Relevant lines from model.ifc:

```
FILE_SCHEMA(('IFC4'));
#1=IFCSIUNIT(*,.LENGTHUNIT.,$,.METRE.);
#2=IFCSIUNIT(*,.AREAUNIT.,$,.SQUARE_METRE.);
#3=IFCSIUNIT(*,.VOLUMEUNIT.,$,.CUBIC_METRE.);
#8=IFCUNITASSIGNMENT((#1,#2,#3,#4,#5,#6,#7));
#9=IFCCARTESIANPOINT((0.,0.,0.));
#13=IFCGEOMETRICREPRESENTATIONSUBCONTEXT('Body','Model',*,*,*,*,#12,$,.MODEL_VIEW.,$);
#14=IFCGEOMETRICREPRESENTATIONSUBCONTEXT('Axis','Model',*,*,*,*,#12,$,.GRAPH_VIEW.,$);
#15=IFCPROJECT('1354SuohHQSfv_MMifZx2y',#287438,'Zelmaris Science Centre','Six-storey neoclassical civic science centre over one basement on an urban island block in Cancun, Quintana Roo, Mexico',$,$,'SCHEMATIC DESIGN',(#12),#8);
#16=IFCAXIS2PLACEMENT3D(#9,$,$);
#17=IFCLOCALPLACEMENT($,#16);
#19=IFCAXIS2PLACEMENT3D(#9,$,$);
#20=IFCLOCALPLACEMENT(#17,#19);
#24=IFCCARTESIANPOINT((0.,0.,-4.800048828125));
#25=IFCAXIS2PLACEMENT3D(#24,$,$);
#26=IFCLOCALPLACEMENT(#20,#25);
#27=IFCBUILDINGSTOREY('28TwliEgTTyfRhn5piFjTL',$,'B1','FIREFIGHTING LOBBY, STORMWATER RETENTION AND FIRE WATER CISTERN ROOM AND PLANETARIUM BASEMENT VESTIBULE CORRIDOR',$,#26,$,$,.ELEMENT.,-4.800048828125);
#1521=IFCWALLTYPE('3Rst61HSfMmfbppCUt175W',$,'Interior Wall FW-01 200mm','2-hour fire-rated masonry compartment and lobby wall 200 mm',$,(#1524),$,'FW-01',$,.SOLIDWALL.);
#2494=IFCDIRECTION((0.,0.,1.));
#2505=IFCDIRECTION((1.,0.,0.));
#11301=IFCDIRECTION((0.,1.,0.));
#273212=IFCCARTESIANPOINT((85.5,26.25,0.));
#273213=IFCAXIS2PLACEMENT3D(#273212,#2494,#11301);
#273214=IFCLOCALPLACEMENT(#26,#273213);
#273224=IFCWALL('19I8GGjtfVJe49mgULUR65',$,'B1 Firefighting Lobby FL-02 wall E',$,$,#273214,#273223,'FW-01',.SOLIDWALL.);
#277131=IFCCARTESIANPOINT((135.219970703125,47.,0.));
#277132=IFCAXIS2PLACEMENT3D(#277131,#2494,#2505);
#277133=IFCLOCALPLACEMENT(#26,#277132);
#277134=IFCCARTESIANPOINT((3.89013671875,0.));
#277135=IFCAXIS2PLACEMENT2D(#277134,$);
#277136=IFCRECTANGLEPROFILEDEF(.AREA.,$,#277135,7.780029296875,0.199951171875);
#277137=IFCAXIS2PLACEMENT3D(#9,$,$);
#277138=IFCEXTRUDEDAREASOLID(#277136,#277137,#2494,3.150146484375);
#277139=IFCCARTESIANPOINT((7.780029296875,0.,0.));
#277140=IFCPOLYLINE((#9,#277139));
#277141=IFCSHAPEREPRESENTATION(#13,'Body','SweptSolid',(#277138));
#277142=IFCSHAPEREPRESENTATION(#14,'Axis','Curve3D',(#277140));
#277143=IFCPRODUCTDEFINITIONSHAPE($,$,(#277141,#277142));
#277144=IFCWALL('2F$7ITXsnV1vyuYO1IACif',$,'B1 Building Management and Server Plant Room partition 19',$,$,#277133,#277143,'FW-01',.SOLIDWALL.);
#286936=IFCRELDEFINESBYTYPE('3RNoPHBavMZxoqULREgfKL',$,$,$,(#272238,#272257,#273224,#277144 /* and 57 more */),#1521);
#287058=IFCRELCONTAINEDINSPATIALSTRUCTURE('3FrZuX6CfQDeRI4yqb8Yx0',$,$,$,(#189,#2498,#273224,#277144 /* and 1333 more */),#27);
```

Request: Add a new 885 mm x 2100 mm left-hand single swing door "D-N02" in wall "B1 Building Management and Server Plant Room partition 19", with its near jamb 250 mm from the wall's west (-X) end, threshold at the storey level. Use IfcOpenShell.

```python
import numpy as np
import ifcopenshell
import ifcopenshell.api.feature
import ifcopenshell.api.geometry
import ifcopenshell.api.root
import ifcopenshell.api.spatial
import ifcopenshell.geom
import ifcopenshell.util.element
import ifcopenshell.util.placement
import ifcopenshell.util.representation
import ifcopenshell.util.shape
import ifcopenshell.util.unit

model = ifcopenshell.open("model.ifc")
unit_scale = ifcopenshell.util.unit.calculate_unit_scale(model)
settings = ifcopenshell.geom.settings()


def volume(element):
    """Net volume in cubic metres, openings subtracted."""
    shape = ifcopenshell.geom.create_shape(settings, element)
    return ifcopenshell.util.shape.get_volume(shape.geometry)


wall = model.by_id(277144)
storey = ifcopenshell.util.element.get_container(wall, ifc_class="IfcBuildingStorey")
context = ifcopenshell.util.representation.get_context(model, "Model", "Body", "MODEL_VIEW")
before = volume(wall)

width, height, from_end, sill = 0.885, 2.1, 0.25, 0.0  # metres

# The wall runs along its own X axis, and the end named is its -X end.
wall_shape = ifcopenshell.geom.create_shape(settings, wall)
x, y, z = ifcopenshell.util.shape.get_vertices(wall_shape.geometry).T
start = x.min() + from_end
face, thickness = float(y.min()), float(y.max() - y.min())
wall_matrix = ifcopenshell.util.placement.get_local_placement(wall.ObjectPlacement)
level = ifcopenshell.util.placement.get_local_placement(storey.ObjectPlacement)[2, 3]


def in_wall(x, y):
    """Placement at x, y metres in the wall's axes, at sill height."""
    matrix = wall_matrix.copy()
    matrix[:, 3] = wall_matrix @ np.array([x / unit_scale, y / unit_scale, 0.0, 1.0])
    matrix[2, 3] = level + sill / unit_scale
    return matrix


# Opening: a box that overshoots both wall faces by 50 mm.
opening = ifcopenshell.api.root.create_entity(model, ifc_class="IfcOpeningElement", predefined_type="OPENING")
box = ifcopenshell.api.geometry.add_wall_representation(
    model, context=context, length=width, height=height, thickness=thickness + 0.1
)
ifcopenshell.api.geometry.assign_representation(model, product=opening, representation=box)
ifcopenshell.api.geometry.edit_object_placement(model, product=opening, matrix=in_wall(start, face - 0.05), is_si=False)
ifcopenshell.api.feature.add_feature(model, feature=opening, element=wall)

door = ifcopenshell.api.root.create_entity(model, ifc_class="IfcDoor", name="D-N02", predefined_type="DOOR")
door.OverallWidth, door.OverallHeight = width / unit_scale, height / unit_scale
door.OperationType = "SINGLE_SWING_LEFT"
body = ifcopenshell.api.geometry.add_door_representation(
    model,
    context=context,
    overall_width=door.OverallWidth,
    overall_height=door.OverallHeight,
    operation_type="SINGLE_SWING_LEFT",
    lining_properties={"LiningDepth": thickness / unit_scale, "ThresholdDepth": thickness / unit_scale},
)
ifcopenshell.api.geometry.assign_representation(model, product=door, representation=body)
ifcopenshell.api.spatial.assign_container(model, products=[door], relating_structure=storey)
ifcopenshell.api.feature.add_filling(model, opening=opening, element=door)

# The lining spans the wall, so the door starts at the wall face.
ifcopenshell.api.geometry.edit_object_placement(model, product=door, matrix=in_wall(start, face), is_si=False)

after = volume(wall)

print(f"wall volume {before:.3f} -> {after:.3f} m3")

model.write("model_v2.ifc")
```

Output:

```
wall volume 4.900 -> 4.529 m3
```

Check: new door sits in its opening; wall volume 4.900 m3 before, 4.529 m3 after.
